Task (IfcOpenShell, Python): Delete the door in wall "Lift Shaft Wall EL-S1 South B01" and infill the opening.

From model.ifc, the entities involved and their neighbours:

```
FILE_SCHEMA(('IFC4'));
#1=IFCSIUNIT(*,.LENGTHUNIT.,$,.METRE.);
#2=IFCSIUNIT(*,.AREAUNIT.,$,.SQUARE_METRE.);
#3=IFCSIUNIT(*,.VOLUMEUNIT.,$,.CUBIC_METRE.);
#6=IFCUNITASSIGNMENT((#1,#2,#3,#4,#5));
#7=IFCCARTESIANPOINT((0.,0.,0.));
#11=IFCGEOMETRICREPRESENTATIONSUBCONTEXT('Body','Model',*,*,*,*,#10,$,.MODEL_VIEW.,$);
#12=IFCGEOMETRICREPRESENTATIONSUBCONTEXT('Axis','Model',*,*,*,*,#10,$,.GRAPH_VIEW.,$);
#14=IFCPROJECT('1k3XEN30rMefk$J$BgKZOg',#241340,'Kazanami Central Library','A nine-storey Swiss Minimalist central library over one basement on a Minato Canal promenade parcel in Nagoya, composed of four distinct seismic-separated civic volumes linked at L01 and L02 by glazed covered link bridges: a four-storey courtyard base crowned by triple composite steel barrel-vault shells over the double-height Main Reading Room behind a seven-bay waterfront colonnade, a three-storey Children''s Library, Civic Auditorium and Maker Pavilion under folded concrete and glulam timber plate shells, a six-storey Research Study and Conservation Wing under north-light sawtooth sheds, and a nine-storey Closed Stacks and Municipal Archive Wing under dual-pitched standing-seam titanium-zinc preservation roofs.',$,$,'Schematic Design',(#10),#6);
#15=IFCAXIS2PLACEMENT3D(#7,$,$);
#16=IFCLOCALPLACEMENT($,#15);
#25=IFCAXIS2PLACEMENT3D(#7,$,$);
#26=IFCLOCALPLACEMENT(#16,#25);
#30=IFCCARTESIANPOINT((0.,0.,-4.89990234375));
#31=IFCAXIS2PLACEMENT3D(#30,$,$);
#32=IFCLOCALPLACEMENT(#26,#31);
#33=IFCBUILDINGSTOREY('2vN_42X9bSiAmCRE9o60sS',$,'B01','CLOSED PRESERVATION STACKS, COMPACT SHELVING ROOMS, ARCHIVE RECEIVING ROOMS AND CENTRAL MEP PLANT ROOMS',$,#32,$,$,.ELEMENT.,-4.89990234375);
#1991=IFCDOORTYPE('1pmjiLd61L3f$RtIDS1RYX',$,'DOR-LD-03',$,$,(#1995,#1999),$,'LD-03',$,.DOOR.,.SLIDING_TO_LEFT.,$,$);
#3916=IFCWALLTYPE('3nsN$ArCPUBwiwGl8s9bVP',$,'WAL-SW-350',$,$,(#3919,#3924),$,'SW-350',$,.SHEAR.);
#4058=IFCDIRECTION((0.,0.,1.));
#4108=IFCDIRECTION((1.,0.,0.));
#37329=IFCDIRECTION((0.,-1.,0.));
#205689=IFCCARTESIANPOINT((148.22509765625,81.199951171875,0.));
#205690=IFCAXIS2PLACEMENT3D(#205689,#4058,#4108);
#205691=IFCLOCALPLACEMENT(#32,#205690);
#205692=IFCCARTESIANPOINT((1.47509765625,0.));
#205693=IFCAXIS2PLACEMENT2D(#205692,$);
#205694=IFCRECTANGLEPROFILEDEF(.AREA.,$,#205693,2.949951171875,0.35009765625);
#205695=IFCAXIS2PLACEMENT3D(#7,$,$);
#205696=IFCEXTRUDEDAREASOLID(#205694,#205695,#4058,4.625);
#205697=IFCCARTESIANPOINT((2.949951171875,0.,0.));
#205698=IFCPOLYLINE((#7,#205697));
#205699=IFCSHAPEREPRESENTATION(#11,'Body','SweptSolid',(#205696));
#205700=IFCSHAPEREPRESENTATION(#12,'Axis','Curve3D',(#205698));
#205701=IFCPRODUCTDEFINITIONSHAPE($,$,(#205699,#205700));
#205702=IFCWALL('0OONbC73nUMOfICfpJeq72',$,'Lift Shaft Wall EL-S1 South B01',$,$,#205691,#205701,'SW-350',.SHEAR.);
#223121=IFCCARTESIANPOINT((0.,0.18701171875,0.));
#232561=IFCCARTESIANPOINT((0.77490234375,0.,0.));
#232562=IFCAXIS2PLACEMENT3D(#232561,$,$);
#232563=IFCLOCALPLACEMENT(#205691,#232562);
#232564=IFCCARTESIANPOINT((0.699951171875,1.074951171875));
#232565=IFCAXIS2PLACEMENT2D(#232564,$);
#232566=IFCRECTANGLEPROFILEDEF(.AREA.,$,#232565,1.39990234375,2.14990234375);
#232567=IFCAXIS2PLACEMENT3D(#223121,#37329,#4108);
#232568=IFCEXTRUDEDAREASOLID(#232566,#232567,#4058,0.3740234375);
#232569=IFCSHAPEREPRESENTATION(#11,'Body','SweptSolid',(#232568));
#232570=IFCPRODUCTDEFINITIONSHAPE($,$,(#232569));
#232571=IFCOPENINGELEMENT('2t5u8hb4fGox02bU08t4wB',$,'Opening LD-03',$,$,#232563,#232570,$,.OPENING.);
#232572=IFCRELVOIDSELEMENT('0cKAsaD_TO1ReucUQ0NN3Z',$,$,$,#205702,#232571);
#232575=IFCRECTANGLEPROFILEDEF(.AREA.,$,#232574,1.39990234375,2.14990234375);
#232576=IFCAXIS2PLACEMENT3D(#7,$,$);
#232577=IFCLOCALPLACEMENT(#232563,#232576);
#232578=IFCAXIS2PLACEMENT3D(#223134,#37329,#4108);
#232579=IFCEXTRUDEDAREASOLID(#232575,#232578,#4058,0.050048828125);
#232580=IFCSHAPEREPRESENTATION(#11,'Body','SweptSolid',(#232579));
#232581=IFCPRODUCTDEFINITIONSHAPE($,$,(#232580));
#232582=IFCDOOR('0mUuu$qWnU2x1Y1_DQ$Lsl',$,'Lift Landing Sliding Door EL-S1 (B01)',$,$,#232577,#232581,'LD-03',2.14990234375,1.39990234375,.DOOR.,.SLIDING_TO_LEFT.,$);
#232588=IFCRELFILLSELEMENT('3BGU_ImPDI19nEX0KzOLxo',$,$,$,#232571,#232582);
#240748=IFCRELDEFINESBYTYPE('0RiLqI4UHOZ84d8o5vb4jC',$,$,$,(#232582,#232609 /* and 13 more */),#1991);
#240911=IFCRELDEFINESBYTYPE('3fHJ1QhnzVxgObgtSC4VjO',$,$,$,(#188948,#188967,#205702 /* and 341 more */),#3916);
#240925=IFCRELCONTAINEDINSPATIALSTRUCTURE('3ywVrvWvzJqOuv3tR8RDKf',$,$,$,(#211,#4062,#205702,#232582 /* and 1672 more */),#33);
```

```python
import ifcopenshell
import ifcopenshell.api.feature
import ifcopenshell.api.root
import ifcopenshell.geom
import ifcopenshell.util.shape

model = ifcopenshell.open("model.ifc")
settings = ifcopenshell.geom.settings()


def volume(element):
    """Net volume in cubic metres, openings subtracted."""
    shape = ifcopenshell.geom.create_shape(settings, element)
    return ifcopenshell.util.shape.get_volume(shape.geometry)


door = model.by_guid("0mUuu$qWnU2x1Y1_DQ$Lsl")
opening = door.FillsVoids[0].RelatingOpeningElement
wall = opening.VoidsElements[0].RelatingBuildingElement
before = volume(wall)

ifcopenshell.api.root.remove_product(model, product=door)
ifcopenshell.api.feature.remove_feature(model, feature=opening)

after = volume(wall)

print(f"wall volume {before:.3f} -> {after:.3f} m3")

model.write("model_rev.ifc")
```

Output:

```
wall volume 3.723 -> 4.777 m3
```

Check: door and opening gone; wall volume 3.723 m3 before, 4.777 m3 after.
